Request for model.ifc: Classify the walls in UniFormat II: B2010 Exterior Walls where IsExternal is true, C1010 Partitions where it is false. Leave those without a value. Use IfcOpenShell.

First a look at what the model holds.

```python
import ifcopenshell
import ifcopenshell.util.element

model = ifcopenshell.open("model.ifc")
print(model.schema)
print("classifications:", [c.Name for c in model.by_type("IfcClassification")])
values = [ifcopenshell.util.element.get_pset(e, "Pset_WallCommon", "IsExternal") for e in model.by_type("IfcWall")]
for value in (True, False, None):
    print("IsExternal", value, values.count(value))
```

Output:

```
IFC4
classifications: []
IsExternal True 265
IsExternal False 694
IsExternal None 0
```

```python
import ifcopenshell
import ifcopenshell.api.classification
import ifcopenshell.util.element

model = ifcopenshell.open("model.ifc")

system = ifcopenshell.api.classification.add_classification(model, classification="UniFormat II")

walls = model.by_type("IfcWall")
external = {e: ifcopenshell.util.element.get_pset(e, "Pset_WallCommon", "IsExternal") for e in walls}
for flag, code, name in ((True, "B2010", "Exterior Walls"), (False, "C1010", "Partitions")):
    products = [e for e in walls if external[e] is flag]
    ifcopenshell.api.classification.add_reference(
        model, products=products, classification=system, identification=code, name=name
    )
    print(code, len(products))

model.write("model_rev.ifc")
```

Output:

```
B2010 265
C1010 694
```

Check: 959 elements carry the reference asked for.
